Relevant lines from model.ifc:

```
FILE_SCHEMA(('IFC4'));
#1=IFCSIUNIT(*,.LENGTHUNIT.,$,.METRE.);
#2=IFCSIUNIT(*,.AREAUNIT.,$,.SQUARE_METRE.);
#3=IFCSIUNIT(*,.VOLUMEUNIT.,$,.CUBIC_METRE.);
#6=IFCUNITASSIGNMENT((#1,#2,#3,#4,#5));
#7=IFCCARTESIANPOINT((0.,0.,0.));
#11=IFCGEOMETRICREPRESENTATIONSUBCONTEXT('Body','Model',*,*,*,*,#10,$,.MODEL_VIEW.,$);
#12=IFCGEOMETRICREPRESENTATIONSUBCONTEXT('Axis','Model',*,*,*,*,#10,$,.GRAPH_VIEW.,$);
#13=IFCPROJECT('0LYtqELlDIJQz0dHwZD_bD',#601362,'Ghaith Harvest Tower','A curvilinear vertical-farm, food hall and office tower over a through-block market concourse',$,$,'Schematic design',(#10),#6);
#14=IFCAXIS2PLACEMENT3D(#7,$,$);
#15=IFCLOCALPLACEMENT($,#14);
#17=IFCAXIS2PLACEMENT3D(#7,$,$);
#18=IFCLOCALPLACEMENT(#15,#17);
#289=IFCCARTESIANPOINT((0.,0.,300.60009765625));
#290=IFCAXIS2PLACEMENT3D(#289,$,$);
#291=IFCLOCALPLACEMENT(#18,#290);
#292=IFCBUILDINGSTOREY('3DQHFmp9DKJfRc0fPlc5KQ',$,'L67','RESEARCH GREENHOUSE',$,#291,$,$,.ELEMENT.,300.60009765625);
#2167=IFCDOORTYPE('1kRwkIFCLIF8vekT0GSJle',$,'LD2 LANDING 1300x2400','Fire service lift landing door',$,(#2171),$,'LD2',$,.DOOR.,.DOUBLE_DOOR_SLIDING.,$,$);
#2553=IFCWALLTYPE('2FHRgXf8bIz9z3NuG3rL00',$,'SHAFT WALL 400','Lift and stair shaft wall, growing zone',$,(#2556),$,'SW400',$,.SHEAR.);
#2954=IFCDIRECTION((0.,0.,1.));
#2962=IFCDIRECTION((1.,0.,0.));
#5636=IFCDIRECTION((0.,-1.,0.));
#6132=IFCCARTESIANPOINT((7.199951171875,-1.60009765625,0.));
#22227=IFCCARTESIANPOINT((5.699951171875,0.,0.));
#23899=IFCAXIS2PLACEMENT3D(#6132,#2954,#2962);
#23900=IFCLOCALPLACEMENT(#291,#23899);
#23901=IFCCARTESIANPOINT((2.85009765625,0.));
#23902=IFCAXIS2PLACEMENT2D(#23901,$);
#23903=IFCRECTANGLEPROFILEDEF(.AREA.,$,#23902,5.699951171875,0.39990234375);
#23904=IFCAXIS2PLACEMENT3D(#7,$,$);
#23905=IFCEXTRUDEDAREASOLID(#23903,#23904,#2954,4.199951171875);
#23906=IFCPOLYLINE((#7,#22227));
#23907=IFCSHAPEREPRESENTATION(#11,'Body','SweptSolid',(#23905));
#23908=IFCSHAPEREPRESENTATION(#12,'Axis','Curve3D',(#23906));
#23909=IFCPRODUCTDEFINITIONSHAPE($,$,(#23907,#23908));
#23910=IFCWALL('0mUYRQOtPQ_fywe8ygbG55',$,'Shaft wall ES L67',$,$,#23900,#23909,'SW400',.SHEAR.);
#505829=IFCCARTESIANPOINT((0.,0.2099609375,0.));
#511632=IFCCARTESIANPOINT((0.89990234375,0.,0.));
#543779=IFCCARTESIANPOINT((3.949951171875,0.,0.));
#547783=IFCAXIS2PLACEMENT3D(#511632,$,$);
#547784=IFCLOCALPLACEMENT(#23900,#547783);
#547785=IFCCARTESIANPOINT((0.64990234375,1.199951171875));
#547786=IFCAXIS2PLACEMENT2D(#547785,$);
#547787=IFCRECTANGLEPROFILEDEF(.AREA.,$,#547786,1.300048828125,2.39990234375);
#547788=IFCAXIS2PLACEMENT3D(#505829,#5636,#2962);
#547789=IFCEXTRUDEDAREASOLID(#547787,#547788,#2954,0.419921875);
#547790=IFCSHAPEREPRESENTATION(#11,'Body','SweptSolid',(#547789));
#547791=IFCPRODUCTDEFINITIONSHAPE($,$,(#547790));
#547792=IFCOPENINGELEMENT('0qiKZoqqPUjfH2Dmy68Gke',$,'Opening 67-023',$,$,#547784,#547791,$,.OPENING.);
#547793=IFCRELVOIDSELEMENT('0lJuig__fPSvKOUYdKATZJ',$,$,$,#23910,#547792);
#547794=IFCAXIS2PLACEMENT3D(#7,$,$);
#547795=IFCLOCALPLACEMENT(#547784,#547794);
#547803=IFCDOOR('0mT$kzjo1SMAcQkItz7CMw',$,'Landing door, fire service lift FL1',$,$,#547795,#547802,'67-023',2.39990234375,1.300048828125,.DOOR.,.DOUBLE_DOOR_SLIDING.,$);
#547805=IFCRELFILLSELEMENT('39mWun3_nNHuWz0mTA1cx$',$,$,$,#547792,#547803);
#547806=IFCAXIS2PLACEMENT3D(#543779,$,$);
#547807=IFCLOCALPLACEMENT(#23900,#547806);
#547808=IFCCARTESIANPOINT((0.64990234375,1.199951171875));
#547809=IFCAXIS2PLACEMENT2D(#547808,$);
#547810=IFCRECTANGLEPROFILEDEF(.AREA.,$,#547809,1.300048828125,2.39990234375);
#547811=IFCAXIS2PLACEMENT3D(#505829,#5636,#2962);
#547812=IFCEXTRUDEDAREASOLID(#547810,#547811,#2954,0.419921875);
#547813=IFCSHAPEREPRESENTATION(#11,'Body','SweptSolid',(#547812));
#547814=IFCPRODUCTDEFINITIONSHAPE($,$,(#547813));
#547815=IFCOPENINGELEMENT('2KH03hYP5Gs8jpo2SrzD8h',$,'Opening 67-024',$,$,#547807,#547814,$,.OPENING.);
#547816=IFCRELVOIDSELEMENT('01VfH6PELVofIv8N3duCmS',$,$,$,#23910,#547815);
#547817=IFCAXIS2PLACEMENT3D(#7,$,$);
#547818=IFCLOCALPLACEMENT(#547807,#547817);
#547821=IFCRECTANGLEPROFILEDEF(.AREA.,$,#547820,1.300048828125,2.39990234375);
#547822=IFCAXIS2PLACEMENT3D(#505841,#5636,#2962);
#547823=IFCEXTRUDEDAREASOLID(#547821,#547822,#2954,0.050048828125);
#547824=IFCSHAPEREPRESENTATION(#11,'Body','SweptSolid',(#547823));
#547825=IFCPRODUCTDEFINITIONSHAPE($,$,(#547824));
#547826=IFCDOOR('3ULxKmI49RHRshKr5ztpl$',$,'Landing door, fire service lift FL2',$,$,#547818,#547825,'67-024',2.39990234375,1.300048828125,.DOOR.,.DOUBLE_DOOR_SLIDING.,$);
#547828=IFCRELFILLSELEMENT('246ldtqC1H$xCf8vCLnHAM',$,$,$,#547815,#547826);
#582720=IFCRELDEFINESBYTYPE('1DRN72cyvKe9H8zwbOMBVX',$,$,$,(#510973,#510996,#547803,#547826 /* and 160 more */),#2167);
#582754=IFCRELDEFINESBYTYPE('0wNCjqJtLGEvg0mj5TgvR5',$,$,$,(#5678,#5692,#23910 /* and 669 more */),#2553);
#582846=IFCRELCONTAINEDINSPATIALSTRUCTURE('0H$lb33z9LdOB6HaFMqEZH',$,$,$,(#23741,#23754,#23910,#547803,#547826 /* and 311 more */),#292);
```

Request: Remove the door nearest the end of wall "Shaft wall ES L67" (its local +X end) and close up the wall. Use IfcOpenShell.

```python
import ifcopenshell
import ifcopenshell.api.feature
import ifcopenshell.api.root
import ifcopenshell.geom
import ifcopenshell.util.shape

model = ifcopenshell.open("model.ifc")
settings = ifcopenshell.geom.settings()


def volume(element):
    """Net volume in cubic metres, openings subtracted."""
    shape = ifcopenshell.geom.create_shape(settings, element)
    return ifcopenshell.util.shape.get_volume(shape.geometry)


door = model.by_guid("3ULxKmI49RHRshKr5ztpl$")
opening = door.FillsVoids[0].RelatingOpeningElement
wall = opening.VoidsElements[0].RelatingBuildingElement
before = volume(wall)

ifcopenshell.api.root.remove_product(model, product=door)
ifcopenshell.api.feature.remove_feature(model, feature=opening)

after = volume(wall)

print(f"wall volume {before:.3f} -> {after:.3f} m3")

model.write("model-out.ifc")
```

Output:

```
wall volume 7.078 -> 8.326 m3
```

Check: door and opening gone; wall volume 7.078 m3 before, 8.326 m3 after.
